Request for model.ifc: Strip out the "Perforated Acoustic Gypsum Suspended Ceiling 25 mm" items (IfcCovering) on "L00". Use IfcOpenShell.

First a look at what the model holds.

```python
import ifcopenshell
import ifcopenshell.util.element

model = ifcopenshell.open("model.ifc")
print(model.schema)
storey = next(s for s in model.by_type("IfcBuildingStorey") if s.Name == "L00")
coverings = [e for e in ifcopenshell.util.element.get_decomposition(storey) if e.is_a("IfcCovering")]
seen = {}
for e in coverings:
    element_type = ifcopenshell.util.element.get_type(e)
    name = element_type.Name if element_type not in (None, e) else None
    seen[name] = seen.get(name, 0) + 1
for name, count in sorted(seen.items(), key=str):
    print(count, "x", name)
```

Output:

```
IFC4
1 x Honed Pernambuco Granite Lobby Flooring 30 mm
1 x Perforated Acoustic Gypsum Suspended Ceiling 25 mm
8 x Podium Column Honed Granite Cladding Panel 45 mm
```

```python
import ifcopenshell
import ifcopenshell.api.root
import ifcopenshell.util.element

model = ifcopenshell.open("model.ifc")

storey = next(s for s in model.by_type("IfcBuildingStorey") if s.Name == "L00")
coverings = [e for e in ifcopenshell.util.element.get_decomposition(storey) if e.is_a("IfcCovering")]
targets = [e for e in coverings if (t := ifcopenshell.util.element.get_type(e)) not in (None, e) and t.Name == "Perforated Acoustic Gypsum Suspended Ceiling 25 mm"]

for e in targets:
    ifcopenshell.api.root.remove_product(model, product=e)
print(len(targets), "removed")

model.write("model-out.ifc")
```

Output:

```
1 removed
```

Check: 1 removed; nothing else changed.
